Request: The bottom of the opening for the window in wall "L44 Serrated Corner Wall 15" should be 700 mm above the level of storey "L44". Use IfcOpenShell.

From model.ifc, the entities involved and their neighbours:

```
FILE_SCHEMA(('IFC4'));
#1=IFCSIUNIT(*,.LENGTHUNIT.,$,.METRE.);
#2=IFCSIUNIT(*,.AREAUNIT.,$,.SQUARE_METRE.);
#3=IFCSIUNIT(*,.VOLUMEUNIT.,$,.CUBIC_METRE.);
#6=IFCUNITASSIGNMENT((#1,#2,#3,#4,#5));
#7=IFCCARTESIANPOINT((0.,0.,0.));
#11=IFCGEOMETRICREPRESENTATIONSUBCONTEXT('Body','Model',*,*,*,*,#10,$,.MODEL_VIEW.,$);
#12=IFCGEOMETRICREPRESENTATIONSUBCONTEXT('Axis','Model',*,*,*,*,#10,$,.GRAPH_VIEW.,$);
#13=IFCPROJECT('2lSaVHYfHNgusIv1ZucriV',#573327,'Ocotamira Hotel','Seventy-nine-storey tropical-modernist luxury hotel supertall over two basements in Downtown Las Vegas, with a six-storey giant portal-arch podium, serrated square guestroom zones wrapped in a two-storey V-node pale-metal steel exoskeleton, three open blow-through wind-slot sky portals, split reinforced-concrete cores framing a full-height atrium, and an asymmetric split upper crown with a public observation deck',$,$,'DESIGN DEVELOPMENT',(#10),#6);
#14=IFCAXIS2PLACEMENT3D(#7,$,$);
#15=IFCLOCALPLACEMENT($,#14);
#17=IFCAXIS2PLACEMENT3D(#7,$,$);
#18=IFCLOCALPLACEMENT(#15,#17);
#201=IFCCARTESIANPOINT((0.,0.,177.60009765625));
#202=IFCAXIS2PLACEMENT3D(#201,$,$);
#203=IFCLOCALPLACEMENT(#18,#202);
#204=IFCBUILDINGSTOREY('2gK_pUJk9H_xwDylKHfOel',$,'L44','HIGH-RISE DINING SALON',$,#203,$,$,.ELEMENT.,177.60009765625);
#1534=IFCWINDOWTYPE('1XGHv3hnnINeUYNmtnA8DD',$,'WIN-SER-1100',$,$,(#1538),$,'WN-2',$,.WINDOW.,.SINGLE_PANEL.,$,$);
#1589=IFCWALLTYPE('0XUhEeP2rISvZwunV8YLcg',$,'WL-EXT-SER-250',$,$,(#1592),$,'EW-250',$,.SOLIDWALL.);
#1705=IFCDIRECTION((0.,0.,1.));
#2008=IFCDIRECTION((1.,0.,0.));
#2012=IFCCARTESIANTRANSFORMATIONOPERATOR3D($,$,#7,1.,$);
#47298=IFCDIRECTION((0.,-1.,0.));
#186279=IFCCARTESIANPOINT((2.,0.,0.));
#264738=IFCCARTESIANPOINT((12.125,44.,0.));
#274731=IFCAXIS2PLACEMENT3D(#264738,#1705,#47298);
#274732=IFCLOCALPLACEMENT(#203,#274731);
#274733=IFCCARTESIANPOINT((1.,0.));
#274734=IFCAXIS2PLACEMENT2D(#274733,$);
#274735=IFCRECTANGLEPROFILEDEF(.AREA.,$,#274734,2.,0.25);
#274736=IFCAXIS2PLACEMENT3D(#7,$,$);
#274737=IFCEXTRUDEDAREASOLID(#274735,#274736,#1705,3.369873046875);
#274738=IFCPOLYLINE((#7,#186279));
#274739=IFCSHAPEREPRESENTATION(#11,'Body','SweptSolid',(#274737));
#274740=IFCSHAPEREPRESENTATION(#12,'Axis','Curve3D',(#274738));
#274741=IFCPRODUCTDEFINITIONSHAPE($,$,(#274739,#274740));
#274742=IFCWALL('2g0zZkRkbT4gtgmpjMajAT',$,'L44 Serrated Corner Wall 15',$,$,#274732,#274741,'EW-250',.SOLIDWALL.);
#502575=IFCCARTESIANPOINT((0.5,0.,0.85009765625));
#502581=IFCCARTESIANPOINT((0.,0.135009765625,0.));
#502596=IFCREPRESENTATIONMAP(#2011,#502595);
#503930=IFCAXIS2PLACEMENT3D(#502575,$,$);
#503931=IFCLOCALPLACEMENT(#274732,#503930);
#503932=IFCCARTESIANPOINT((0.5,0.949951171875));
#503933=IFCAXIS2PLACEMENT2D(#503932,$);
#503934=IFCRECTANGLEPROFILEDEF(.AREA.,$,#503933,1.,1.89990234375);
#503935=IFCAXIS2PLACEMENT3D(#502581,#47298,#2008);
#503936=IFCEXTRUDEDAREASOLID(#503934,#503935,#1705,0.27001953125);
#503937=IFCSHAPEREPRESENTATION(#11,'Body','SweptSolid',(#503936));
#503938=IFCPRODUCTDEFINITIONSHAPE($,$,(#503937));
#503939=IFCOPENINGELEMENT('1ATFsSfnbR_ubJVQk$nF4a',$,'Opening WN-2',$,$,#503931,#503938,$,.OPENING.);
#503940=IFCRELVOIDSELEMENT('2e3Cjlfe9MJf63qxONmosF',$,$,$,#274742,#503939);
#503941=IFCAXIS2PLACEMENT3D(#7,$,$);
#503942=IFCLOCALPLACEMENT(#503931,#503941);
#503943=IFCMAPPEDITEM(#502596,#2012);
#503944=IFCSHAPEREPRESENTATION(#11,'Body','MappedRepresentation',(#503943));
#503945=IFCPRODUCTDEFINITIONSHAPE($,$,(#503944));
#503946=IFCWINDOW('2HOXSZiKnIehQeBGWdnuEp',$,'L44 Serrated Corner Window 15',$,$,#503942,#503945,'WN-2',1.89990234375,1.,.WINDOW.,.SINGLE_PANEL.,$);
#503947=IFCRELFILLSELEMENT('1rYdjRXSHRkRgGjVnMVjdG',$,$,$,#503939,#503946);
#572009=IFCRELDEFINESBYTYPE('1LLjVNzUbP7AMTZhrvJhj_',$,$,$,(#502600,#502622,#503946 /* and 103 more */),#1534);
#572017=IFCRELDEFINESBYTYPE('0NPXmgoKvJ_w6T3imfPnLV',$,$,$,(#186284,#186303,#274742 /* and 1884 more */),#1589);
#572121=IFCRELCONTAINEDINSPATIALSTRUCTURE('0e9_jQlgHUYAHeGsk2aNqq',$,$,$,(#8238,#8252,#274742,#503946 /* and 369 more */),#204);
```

```python
import numpy as np
import ifcopenshell
import ifcopenshell.api.geometry
import ifcopenshell.geom
import ifcopenshell.util.element
import ifcopenshell.util.placement
import ifcopenshell.util.shape
import ifcopenshell.util.unit

model = ifcopenshell.open("model.ifc")
unit_scale = ifcopenshell.util.unit.calculate_unit_scale(model)

window = model.by_guid("2HOXSZiKnIehQeBGWdnuEp")
opening = window.FillsVoids[0].RelatingOpeningElement
storey = ifcopenshell.util.element.get_container(window, ifc_class="IfcBuildingStorey")
level = ifcopenshell.util.placement.get_local_placement(storey.ObjectPlacement)[2, 3]

# The opening's origin need not be at the sill, so measure its lowest point.
shape = ifcopenshell.geom.create_shape(ifcopenshell.geom.settings(), opening)
bottom = ifcopenshell.util.shape.get_shape_bottom_elevation(shape, shape.geometry) / unit_scale
dz = level + 0.7 - bottom

shift = np.array([0.0, 0.0, dz])
# The window is placed relative to its opening, so it follows when the opening moves.
matrix = ifcopenshell.util.placement.get_local_placement(opening.ObjectPlacement)
matrix[:3, 3] += shift
ifcopenshell.api.geometry.edit_object_placement(
    model, product=opening, matrix=matrix, is_si=False, should_transform_children=True
)

print(f"moved by {dz * unit_scale:+.3f} m")

model.write("model-out.ifc")
```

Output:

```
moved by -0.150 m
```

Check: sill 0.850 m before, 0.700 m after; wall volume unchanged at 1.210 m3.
